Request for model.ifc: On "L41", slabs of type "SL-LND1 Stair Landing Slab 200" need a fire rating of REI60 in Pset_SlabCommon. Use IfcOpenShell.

First a look at what the model holds.

```python
import ifcopenshell
import ifcopenshell.util.element

model = ifcopenshell.open("model.ifc")
print(model.schema)
storey = next(s for s in model.by_type("IfcBuildingStorey") if s.Name == "L41")
slabs = [e for e in ifcopenshell.util.element.get_decomposition(storey) if e.is_a("IfcSlab")]
seen = {}
for e in slabs:
    element_type = ifcopenshell.util.element.get_type(e)
    key = (element_type.Name if element_type != e and element_type else None, ifcopenshell.util.element.get_pset(e, "Pset_SlabCommon", "FireRating"))
    seen[key] = seen.get(key, 0) + 1
for (name, value), count in sorted(seen.items(), key=str):
    print(count, "x", name, "|", value)
```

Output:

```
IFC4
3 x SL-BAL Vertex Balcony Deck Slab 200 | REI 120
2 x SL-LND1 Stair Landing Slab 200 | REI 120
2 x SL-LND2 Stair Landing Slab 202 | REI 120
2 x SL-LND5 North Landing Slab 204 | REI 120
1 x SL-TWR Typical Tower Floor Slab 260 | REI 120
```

```python
import ifcopenshell
import ifcopenshell.api.pset
import ifcopenshell.util.element

model = ifcopenshell.open("model.ifc")

storey = next(s for s in model.by_type("IfcBuildingStorey") if s.Name == "L41")
slabs = [e for e in ifcopenshell.util.element.get_decomposition(storey) if e.is_a("IfcSlab")]

count = 0
for e in slabs:
    element_type = ifcopenshell.util.element.get_type(e)
    if element_type in (None, e) or element_type.Name != "SL-LND1 Stair Landing Slab 200":
        continue
    found = ifcopenshell.util.element.get_pset(e, "Pset_SlabCommon", should_inherit=False)
    if found:
        pset = model.by_id(found["id"])
        if len(ifcopenshell.util.element.get_elements_by_pset(pset)) > 1:
            pset = ifcopenshell.api.pset.unshare_pset(model, products=[e], pset=pset)[0]
    else:
        pset = ifcopenshell.api.pset.add_pset(model, product=e, name="Pset_SlabCommon")
    ifcopenshell.api.pset.edit_pset(model, pset=pset, properties={"FireRating": "REI60"})
    count += 1

print(count, "slabs updated")

model.write("model-out.ifc")
```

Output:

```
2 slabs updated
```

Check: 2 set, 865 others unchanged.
